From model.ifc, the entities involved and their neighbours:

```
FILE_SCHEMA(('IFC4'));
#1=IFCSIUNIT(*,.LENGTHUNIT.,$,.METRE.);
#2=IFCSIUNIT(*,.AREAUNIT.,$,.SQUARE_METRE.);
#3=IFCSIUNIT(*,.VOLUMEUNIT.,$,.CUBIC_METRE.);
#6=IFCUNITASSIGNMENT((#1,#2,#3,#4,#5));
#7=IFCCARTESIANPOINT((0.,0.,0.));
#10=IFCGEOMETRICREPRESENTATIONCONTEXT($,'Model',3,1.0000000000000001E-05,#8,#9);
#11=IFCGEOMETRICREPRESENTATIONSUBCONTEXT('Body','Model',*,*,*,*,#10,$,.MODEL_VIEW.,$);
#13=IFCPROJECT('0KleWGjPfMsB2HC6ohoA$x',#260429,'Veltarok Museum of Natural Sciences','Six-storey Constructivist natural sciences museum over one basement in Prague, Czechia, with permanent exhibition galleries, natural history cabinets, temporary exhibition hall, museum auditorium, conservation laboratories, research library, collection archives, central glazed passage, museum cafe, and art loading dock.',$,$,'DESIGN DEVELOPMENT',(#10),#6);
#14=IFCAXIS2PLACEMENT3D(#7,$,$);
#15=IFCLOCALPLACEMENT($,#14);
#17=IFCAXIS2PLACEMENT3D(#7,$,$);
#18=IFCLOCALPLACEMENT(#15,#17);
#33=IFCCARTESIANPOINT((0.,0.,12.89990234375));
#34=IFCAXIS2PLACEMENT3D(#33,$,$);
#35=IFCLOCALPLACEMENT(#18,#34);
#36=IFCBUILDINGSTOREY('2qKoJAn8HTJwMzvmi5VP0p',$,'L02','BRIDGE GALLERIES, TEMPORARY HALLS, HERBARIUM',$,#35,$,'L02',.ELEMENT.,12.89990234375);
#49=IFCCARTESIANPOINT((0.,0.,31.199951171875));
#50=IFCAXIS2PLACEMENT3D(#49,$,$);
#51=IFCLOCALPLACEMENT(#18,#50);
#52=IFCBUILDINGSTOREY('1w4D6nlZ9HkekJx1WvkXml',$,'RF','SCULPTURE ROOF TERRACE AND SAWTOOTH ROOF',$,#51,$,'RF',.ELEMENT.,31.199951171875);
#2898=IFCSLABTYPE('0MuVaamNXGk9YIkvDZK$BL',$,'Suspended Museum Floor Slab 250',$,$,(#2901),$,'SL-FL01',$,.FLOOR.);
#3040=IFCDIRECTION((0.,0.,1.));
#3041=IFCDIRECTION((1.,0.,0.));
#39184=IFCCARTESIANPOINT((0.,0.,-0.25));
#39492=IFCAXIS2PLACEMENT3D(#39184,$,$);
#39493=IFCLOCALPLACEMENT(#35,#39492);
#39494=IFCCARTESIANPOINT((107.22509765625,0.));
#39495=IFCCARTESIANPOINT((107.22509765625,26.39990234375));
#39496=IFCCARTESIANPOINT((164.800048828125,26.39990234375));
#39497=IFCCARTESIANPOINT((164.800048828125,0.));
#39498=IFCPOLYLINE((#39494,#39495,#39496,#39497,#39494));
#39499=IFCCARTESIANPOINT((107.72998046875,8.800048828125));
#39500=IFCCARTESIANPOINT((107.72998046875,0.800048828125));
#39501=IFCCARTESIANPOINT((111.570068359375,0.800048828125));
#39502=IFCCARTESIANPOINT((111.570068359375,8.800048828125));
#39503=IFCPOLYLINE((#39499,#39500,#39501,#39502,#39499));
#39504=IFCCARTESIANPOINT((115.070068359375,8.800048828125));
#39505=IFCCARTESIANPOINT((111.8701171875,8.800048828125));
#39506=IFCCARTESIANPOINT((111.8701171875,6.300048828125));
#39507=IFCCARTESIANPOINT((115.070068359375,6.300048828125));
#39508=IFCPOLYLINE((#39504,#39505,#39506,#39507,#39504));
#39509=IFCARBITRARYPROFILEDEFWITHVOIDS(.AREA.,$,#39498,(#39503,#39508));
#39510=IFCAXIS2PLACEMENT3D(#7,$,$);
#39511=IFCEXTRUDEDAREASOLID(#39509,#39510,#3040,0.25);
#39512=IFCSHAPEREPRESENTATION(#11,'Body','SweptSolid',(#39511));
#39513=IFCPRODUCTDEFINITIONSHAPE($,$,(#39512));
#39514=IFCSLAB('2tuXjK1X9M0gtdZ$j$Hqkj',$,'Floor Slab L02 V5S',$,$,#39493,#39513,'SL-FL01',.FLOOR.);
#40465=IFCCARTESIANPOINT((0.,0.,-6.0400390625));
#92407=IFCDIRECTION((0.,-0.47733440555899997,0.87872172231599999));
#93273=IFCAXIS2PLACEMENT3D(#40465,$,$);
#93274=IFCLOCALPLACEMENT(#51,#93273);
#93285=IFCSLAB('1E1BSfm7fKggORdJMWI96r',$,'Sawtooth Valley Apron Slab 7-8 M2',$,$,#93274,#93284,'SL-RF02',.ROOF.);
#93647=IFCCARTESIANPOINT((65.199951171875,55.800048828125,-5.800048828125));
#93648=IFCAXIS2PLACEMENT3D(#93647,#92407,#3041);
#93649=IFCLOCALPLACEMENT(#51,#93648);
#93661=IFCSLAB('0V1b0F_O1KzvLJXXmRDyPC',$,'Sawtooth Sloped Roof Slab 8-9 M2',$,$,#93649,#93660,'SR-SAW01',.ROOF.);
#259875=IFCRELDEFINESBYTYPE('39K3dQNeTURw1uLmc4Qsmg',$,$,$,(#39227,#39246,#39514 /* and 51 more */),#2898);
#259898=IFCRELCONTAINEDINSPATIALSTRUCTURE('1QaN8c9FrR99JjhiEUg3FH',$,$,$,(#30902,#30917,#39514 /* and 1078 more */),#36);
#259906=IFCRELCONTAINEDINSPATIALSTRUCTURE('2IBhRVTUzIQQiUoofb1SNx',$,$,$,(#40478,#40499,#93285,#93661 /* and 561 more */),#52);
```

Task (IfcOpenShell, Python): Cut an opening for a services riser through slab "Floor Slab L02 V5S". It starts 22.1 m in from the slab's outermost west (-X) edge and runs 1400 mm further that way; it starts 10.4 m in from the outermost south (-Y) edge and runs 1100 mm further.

```python
import numpy as np
import ifcopenshell
import ifcopenshell.api.feature
import ifcopenshell.api.geometry
import ifcopenshell.api.root
import ifcopenshell.geom
import ifcopenshell.util.placement
import ifcopenshell.util.representation
import ifcopenshell.util.shape
import ifcopenshell.util.unit

model = ifcopenshell.open("model.ifc")
unit_scale = ifcopenshell.util.unit.calculate_unit_scale(model)
settings = ifcopenshell.geom.settings()


def volume(element):
    """Net volume in cubic metres, openings subtracted."""
    shape = ifcopenshell.geom.create_shape(settings, element)
    return ifcopenshell.util.shape.get_volume(shape.geometry)


slab = model.by_guid("2tuXjK1X9M0gtdZ$j$Hqkj")
before = volume(slab)

# Extent in the slab's own axes, in metres. The edges named are its -X and -Y sides.
slab_shape = ifcopenshell.geom.create_shape(settings, slab)
vertices = ifcopenshell.util.shape.get_vertices(slab_shape.geometry)
x_min, y_min, bottom = vertices.min(axis=0)
top = vertices[:, 2].max()

opening = ifcopenshell.api.root.create_entity(model, ifc_class="IfcOpeningElement", name="Services riser opening", predefined_type="OPENING")
context = ifcopenshell.util.representation.get_context(model, "Model", "Body", "MODEL_VIEW")
width, depth = 1.4, 1.1
outline = [(0.0, 0.0), (width, 0.0), (width, depth), (0.0, depth), (0.0, 0.0)]
# Overshoot both faces by 50 mm so the cut is clean.
shape = ifcopenshell.api.geometry.add_slab_representation(
    model, context=context, depth=top - bottom + 0.1, polyline=outline
)
ifcopenshell.api.geometry.assign_representation(model, product=opening, representation=shape)

matrix = ifcopenshell.util.placement.get_local_placement(slab.ObjectPlacement)
matrix[:, 3] = matrix @ np.append(np.array([x_min + 22.1, y_min + 10.4, bottom - 0.05]) / unit_scale, 1.0)
ifcopenshell.api.geometry.edit_object_placement(model, product=opening, matrix=matrix, is_si=False)
ifcopenshell.api.feature.add_feature(model, feature=opening, element=slab)

after = volume(slab)

print(f"slab volume {before:.3f} -> {after:.3f} m3")

model.write("model_v2.ifc")
```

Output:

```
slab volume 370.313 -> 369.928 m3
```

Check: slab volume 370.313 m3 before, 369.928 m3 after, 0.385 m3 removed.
